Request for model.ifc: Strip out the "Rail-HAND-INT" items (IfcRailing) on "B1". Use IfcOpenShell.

First a look at what the model holds.

```python
import ifcopenshell
import ifcopenshell.util.element

model = ifcopenshell.open("model.ifc")
print(model.schema)
storey = next(s for s in model.by_type("IfcBuildingStorey") if s.Name == "B1")
railings = [e for e in ifcopenshell.util.element.get_decomposition(storey) if e.is_a("IfcRailing")]
seen = {}
for e in railings:
    element_type = ifcopenshell.util.element.get_type(e)
    name = element_type.Name if element_type not in (None, e) else None
    seen[name] = seen.get(name, 0) + 1
for name, count in sorted(seen.items(), key=str):
    print(count, "x", name)
```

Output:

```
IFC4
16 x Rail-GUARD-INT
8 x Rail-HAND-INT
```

```python
import ifcopenshell
import ifcopenshell.api.root
import ifcopenshell.util.element

model = ifcopenshell.open("model.ifc")

storey = next(s for s in model.by_type("IfcBuildingStorey") if s.Name == "B1")
railings = [e for e in ifcopenshell.util.element.get_decomposition(storey) if e.is_a("IfcRailing")]
targets = [e for e in railings if (t := ifcopenshell.util.element.get_type(e)) not in (None, e) and t.Name == "Rail-HAND-INT"]

for e in targets:
    ifcopenshell.api.root.remove_product(model, product=e)
print(len(targets), "removed")

model.write("model_v2.ifc")
```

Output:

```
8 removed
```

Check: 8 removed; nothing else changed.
